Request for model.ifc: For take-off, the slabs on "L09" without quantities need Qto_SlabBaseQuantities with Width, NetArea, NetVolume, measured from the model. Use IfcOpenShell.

First a look at what the model holds.

```python
import ifcopenshell
import ifcopenshell.util.element
import ifcopenshell.util.unit

model = ifcopenshell.open("model.ifc")
print(model.schema)
for unit_type in ("LENGTHUNIT", "AREAUNIT", "VOLUMEUNIT"):
    print(unit_type, ifcopenshell.util.unit.calculate_unit_scale(model, unit_type))
storey = next(s for s in model.by_type("IfcBuildingStorey") if s.Name == "L09")
slabs = [e for e in ifcopenshell.util.element.get_decomposition(storey) if e.is_a("IfcSlab")]
for e in sorted(slabs, key=lambda e: e.id()):
    print(e.id(), e.is_a(), e.Name, list(ifcopenshell.util.element.get_psets(e, qtos_only=True)), sep=" | ")
```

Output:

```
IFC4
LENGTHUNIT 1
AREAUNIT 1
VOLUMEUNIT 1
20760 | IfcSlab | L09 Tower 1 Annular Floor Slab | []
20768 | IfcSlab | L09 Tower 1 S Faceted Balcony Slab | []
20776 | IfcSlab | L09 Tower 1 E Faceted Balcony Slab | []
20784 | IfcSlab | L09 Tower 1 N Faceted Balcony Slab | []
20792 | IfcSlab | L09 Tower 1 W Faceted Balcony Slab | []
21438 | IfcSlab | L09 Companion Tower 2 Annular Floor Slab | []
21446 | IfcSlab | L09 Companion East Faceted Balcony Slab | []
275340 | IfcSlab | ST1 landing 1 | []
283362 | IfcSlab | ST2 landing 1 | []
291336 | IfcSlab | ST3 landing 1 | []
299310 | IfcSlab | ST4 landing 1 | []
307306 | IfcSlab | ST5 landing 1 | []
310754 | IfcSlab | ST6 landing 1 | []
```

```python
import ifcopenshell
import ifcopenshell.api.pset
import ifcopenshell.geom
import ifcopenshell.util.element
import ifcopenshell.util.shape
import ifcopenshell.util.unit

model = ifcopenshell.open("model.ifc")
unit_scale = ifcopenshell.util.unit.calculate_unit_scale(model)
area_scale = ifcopenshell.util.unit.calculate_unit_scale(model, "AREAUNIT")
volume_scale = ifcopenshell.util.unit.calculate_unit_scale(model, "VOLUMEUNIT")
settings = ifcopenshell.geom.settings()

storey = next(s for s in model.by_type("IfcBuildingStorey") if s.Name == "L09")
slabs = [e for e in ifcopenshell.util.element.get_decomposition(storey) if e.is_a("IfcSlab")]

for e in sorted(slabs, key=lambda e: e.id()):
    if ifcopenshell.util.element.get_psets(e, qtos_only=True, should_inherit=False):
        continue
    # Geometry comes back in metres, in the element's own axes.
    shape = ifcopenshell.geom.create_shape(settings, e)
    values = {
        "Width": ifcopenshell.util.shape.get_z(shape.geometry) / unit_scale,
        "NetArea": ifcopenshell.util.shape.get_footprint_area(shape.geometry) / area_scale,
        "NetVolume": ifcopenshell.util.shape.get_volume(shape.geometry) / volume_scale,
    }
    qto = ifcopenshell.api.pset.add_qto(model, product=e, name="Qto_SlabBaseQuantities")
    ifcopenshell.api.pset.edit_qto(model, qto=qto, properties=values)
    print(e.id(), {k: round(v, 3) for k, v in values.items()})

model.write("model_v2.ifc")
```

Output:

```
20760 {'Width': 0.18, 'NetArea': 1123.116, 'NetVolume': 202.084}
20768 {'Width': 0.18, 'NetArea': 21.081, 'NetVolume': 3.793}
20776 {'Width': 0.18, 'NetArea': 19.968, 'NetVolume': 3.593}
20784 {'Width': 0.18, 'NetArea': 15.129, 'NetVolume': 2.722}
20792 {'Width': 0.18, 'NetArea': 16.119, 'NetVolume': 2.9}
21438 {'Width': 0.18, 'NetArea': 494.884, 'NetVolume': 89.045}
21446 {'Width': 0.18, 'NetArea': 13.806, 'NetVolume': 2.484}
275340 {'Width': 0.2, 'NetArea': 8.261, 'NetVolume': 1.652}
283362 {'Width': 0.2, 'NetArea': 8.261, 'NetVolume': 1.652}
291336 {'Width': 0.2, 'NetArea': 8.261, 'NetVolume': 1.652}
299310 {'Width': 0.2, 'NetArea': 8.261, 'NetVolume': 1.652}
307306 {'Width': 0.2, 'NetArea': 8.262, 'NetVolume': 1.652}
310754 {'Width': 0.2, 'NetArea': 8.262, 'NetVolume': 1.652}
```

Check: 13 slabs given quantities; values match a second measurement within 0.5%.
